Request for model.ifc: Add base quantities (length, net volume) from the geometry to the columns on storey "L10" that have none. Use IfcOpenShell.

First a look at what the model holds.

```python
import ifcopenshell
import ifcopenshell.util.element
import ifcopenshell.util.unit

model = ifcopenshell.open("model.ifc")
print(model.schema)
for unit_type in ("LENGTHUNIT", "AREAUNIT", "VOLUMEUNIT"):
    print(unit_type, ifcopenshell.util.unit.calculate_unit_scale(model, unit_type))
storey = next(s for s in model.by_type("IfcBuildingStorey") if s.Name == "L10")
columns = [e for e in ifcopenshell.util.element.get_decomposition(storey) if e.is_a("IfcColumn")]
for e in sorted(columns, key=lambda e: e.id()):
    print(e.id(), e.is_a(), e.Name, list(ifcopenshell.util.element.get_psets(e, qtos_only=True)), sep=" | ")
```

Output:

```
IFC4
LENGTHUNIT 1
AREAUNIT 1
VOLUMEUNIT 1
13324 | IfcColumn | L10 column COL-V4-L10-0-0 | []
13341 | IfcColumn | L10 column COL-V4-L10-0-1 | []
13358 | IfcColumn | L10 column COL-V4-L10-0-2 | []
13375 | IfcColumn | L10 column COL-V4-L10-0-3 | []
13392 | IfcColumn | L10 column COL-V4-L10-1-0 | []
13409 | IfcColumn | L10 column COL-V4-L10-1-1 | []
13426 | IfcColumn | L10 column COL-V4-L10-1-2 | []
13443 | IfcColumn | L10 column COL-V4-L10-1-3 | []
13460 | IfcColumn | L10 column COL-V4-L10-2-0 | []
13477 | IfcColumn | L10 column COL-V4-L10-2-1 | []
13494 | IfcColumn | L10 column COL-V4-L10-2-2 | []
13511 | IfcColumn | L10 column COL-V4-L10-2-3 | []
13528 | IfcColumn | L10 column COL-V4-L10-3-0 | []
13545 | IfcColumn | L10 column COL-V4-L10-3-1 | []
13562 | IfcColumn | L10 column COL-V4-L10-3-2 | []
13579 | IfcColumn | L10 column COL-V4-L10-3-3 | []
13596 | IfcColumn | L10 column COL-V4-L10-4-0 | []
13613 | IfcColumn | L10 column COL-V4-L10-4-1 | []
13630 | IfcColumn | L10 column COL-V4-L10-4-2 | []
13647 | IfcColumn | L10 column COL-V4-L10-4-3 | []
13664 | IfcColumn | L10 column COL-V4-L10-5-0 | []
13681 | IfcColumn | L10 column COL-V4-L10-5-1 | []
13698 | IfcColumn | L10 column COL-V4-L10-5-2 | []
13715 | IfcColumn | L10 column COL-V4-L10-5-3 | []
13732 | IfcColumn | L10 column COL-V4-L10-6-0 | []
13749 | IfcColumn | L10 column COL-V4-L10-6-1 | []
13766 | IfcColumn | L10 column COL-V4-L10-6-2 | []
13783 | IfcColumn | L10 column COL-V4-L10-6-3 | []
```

```python
import ifcopenshell
import ifcopenshell.api.pset
import ifcopenshell.geom
import ifcopenshell.util.element
import ifcopenshell.util.shape
import ifcopenshell.util.unit

model = ifcopenshell.open("model.ifc")
unit_scale = ifcopenshell.util.unit.calculate_unit_scale(model)
volume_scale = ifcopenshell.util.unit.calculate_unit_scale(model, "VOLUMEUNIT")
settings = ifcopenshell.geom.settings()

storey = next(s for s in model.by_type("IfcBuildingStorey") if s.Name == "L10")
columns = [e for e in ifcopenshell.util.element.get_decomposition(storey) if e.is_a("IfcColumn")]

for e in sorted(columns, key=lambda e: e.id()):
    if ifcopenshell.util.element.get_psets(e, qtos_only=True, should_inherit=False):
        continue
    # Geometry comes back in metres, in the element's own axes.
    shape = ifcopenshell.geom.create_shape(settings, e)
    values = {
        "Length": ifcopenshell.util.shape.get_z(shape.geometry) / unit_scale,
        "NetVolume": ifcopenshell.util.shape.get_volume(shape.geometry) / volume_scale,
    }
    qto = ifcopenshell.api.pset.add_qto(model, product=e, name="Qto_ColumnBaseQuantities")
    ifcopenshell.api.pset.edit_qto(model, qto=qto, properties=values)
    print(e.id(), {k: round(v, 3) for k, v in values.items()})

model.write("model_edited.ifc")
```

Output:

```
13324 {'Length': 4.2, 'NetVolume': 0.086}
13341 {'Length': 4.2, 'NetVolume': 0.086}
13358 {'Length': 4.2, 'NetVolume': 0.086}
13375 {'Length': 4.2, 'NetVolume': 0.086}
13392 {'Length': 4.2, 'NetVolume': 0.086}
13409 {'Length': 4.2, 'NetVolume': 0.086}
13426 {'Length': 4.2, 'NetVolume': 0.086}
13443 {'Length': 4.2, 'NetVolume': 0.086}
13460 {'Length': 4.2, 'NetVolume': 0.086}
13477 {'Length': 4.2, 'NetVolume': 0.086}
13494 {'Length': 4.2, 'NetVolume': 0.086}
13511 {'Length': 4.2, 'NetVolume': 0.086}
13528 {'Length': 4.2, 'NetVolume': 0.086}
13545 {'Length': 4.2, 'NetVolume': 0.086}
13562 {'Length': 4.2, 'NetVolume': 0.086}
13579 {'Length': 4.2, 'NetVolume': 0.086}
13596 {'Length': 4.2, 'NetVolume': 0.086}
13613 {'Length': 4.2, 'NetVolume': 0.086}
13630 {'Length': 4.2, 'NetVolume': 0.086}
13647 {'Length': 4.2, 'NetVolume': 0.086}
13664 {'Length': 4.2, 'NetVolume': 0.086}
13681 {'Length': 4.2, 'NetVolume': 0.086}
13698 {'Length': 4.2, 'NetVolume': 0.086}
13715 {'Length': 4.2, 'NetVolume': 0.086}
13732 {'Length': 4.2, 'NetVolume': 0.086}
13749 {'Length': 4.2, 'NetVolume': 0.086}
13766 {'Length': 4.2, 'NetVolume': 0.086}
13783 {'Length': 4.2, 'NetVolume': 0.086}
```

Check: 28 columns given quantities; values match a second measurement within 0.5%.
